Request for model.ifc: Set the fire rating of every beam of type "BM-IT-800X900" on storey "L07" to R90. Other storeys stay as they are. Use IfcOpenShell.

First a look at what the model holds.

```python
import ifcopenshell
import ifcopenshell.util.element

model = ifcopenshell.open("model.ifc")
print(model.schema)
storey = next(s for s in model.by_type("IfcBuildingStorey") if s.Name == "L07")
beams = [e for e in ifcopenshell.util.element.get_decomposition(storey) if e.is_a("IfcBeam")]
seen = {}
for e in beams:
    element_type = ifcopenshell.util.element.get_type(e)
    key = (element_type.Name if element_type != e and element_type else None, ifcopenshell.util.element.get_pset(e, "Pset_BeamCommon", "FireRating"))
    seen[key] = seen.get(key, 0) + 1
for (name, value), count in sorted(seen.items(), key=str):
    print(count, "x", name, "|", value)
```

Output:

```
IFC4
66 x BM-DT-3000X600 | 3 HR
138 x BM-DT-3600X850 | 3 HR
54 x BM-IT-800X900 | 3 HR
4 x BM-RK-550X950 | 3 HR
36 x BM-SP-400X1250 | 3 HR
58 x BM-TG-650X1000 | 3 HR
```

```python
import ifcopenshell
import ifcopenshell.api.pset
import ifcopenshell.util.element

model = ifcopenshell.open("model.ifc")

storey = next(s for s in model.by_type("IfcBuildingStorey") if s.Name == "L07")
beams = [e for e in ifcopenshell.util.element.get_decomposition(storey) if e.is_a("IfcBeam")]

count = 0
for e in beams:
    element_type = ifcopenshell.util.element.get_type(e)
    if element_type in (None, e) or element_type.Name != "BM-IT-800X900":
        continue
    # add_pset returns the element's existing set when there is one.
    pset = ifcopenshell.api.pset.add_pset(model, product=e, name="Pset_BeamCommon")
    ifcopenshell.api.pset.edit_pset(model, pset=pset, properties={"FireRating": "R90"})
    count += 1

print(count, "beams updated")

model.write("model-out.ifc")
```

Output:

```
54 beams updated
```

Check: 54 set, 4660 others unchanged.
